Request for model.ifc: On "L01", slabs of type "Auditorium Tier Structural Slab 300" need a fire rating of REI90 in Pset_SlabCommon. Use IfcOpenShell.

First a look at what the model holds.

```python
import ifcopenshell
import ifcopenshell.util.element

model = ifcopenshell.open("model.ifc")
print(model.schema)
storey = next(s for s in model.by_type("IfcBuildingStorey") if s.Name == "L01")
slabs = [e for e in ifcopenshell.util.element.get_decomposition(storey) if e.is_a("IfcSlab")]
seen = {}
for e in slabs:
    element_type = ifcopenshell.util.element.get_type(e)
    key = (element_type.Name if element_type != e and element_type else None, ifcopenshell.util.element.get_pset(e, "Pset_SlabCommon", "FireRating"))
    seen[key] = seen.get(key, 0) + 1
for (name, value), count in sorted(seen.items(), key=str):
    print(count, "x", name, "|", value)
```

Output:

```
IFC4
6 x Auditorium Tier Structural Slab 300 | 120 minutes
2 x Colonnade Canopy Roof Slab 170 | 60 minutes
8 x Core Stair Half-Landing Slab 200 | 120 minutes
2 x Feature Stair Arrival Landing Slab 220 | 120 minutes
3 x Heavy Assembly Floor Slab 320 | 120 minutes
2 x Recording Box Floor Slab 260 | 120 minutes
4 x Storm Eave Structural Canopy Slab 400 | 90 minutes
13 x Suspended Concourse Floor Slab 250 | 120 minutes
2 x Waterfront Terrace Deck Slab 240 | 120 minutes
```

```python
import ifcopenshell
import ifcopenshell.api.pset
import ifcopenshell.util.element

model = ifcopenshell.open("model.ifc")

storey = next(s for s in model.by_type("IfcBuildingStorey") if s.Name == "L01")
slabs = [e for e in ifcopenshell.util.element.get_decomposition(storey) if e.is_a("IfcSlab")]

count = 0
for e in slabs:
    element_type = ifcopenshell.util.element.get_type(e)
    if element_type in (None, e) or element_type.Name != "Auditorium Tier Structural Slab 300":
        continue
    # add_pset returns the element's existing set when there is one.
    pset = ifcopenshell.api.pset.add_pset(model, product=e, name="Pset_SlabCommon")
    ifcopenshell.api.pset.edit_pset(model, pset=pset, properties={"FireRating": "REI90"})
    count += 1

print(count, "slabs updated")

model.write("model_updated.ifc")
```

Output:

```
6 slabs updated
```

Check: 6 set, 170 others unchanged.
